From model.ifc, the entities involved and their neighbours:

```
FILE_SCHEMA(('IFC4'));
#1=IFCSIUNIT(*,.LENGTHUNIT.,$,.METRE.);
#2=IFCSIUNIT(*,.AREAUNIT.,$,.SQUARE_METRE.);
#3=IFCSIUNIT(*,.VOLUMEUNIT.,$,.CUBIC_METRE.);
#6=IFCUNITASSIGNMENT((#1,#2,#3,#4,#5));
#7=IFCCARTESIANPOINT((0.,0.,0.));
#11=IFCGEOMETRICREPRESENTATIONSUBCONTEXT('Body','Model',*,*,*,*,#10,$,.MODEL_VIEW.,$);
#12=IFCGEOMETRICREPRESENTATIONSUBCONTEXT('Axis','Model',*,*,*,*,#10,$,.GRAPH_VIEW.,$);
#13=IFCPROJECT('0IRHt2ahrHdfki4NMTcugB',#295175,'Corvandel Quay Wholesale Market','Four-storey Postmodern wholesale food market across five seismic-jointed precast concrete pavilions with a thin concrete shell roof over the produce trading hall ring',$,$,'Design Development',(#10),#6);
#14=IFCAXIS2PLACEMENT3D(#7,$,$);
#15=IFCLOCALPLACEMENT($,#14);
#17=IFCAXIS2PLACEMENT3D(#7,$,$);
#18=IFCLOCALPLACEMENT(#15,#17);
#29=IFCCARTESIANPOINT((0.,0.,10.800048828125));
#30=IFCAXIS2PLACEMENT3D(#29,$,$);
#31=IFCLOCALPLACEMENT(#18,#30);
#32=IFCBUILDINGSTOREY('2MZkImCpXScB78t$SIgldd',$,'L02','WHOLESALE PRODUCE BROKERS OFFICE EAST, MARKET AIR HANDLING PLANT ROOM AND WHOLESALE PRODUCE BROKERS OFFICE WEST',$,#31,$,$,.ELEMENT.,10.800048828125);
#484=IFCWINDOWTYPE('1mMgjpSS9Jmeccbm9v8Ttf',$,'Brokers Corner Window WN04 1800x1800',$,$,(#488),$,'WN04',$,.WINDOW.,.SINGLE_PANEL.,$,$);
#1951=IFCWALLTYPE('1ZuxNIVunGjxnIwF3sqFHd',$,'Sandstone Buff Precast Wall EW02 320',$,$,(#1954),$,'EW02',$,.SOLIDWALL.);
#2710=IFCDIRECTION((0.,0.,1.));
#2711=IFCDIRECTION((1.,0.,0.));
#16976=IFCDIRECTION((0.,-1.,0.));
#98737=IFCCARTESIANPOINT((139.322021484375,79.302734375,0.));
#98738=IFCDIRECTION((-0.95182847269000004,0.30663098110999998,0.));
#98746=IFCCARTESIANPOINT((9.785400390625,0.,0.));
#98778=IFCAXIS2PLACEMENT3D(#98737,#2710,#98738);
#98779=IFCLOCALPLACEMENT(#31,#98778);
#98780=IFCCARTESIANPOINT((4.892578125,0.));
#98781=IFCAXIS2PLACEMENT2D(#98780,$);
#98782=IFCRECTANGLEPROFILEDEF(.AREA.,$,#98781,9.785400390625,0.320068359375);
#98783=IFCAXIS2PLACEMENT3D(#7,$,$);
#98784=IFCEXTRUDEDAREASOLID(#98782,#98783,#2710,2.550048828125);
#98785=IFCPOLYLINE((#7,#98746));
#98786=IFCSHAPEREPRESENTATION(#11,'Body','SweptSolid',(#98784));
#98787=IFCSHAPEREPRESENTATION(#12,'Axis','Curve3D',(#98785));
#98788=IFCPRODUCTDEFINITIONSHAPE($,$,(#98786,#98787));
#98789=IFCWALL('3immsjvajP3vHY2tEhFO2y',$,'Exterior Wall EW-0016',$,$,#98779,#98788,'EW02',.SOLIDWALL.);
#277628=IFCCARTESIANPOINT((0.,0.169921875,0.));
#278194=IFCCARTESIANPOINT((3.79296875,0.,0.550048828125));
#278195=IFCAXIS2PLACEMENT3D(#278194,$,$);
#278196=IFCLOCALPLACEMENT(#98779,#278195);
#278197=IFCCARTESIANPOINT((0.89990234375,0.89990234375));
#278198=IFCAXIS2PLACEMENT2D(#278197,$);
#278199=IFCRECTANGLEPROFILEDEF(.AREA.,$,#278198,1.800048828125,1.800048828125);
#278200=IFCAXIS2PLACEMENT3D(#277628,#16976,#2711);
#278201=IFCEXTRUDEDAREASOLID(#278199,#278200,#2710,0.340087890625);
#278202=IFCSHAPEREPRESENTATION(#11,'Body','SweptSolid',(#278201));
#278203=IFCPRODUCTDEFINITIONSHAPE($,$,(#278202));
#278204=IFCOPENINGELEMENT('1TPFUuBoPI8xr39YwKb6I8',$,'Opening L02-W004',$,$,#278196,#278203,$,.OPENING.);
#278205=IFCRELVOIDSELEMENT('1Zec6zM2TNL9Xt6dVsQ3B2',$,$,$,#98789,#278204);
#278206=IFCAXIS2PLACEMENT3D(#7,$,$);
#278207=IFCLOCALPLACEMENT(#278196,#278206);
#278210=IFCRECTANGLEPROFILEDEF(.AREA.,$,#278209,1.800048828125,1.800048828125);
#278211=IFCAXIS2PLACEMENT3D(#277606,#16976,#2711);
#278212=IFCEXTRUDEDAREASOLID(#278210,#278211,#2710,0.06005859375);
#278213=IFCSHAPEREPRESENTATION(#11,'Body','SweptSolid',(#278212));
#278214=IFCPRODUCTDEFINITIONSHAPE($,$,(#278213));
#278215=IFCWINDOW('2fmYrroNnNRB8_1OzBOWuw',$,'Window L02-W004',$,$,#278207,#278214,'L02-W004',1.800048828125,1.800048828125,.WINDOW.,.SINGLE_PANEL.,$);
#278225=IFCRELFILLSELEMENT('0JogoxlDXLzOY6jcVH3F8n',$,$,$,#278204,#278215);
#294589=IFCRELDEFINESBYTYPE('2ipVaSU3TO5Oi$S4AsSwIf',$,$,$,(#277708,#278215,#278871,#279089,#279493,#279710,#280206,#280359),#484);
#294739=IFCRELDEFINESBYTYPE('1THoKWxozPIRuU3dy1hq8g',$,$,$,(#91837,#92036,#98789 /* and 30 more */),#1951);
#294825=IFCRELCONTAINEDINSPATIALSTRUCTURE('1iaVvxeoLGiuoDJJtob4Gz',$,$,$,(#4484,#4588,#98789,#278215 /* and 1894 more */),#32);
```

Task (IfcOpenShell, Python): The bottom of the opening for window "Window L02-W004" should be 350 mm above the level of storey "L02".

```python
import numpy as np
import ifcopenshell
import ifcopenshell.api.geometry
import ifcopenshell.geom
import ifcopenshell.util.element
import ifcopenshell.util.placement
import ifcopenshell.util.shape
import ifcopenshell.util.unit

model = ifcopenshell.open("model.ifc")
unit_scale = ifcopenshell.util.unit.calculate_unit_scale(model)

window = model.by_id(278215)
opening = window.FillsVoids[0].RelatingOpeningElement
storey = ifcopenshell.util.element.get_container(window, ifc_class="IfcBuildingStorey")
level = ifcopenshell.util.placement.get_local_placement(storey.ObjectPlacement)[2, 3]

# The opening's origin need not be at the sill, so measure its lowest point.
shape = ifcopenshell.geom.create_shape(ifcopenshell.geom.settings(), opening)
bottom = ifcopenshell.util.shape.get_shape_bottom_elevation(shape, shape.geometry) / unit_scale
dz = level + 0.35 / unit_scale - bottom

shift = np.array([0.0, 0.0, dz])
# The window is placed relative to its opening, so it follows when the opening moves.
matrix = ifcopenshell.util.placement.get_local_placement(opening.ObjectPlacement)
matrix[:3, 3] += shift
ifcopenshell.api.geometry.edit_object_placement(
    model, product=opening, matrix=matrix, is_si=False, should_transform_children=True
)

print(f"moved by {dz * unit_scale:+.3f} m")

model.write("model_rev.ifc")
```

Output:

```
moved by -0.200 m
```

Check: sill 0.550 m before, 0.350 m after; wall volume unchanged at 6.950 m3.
